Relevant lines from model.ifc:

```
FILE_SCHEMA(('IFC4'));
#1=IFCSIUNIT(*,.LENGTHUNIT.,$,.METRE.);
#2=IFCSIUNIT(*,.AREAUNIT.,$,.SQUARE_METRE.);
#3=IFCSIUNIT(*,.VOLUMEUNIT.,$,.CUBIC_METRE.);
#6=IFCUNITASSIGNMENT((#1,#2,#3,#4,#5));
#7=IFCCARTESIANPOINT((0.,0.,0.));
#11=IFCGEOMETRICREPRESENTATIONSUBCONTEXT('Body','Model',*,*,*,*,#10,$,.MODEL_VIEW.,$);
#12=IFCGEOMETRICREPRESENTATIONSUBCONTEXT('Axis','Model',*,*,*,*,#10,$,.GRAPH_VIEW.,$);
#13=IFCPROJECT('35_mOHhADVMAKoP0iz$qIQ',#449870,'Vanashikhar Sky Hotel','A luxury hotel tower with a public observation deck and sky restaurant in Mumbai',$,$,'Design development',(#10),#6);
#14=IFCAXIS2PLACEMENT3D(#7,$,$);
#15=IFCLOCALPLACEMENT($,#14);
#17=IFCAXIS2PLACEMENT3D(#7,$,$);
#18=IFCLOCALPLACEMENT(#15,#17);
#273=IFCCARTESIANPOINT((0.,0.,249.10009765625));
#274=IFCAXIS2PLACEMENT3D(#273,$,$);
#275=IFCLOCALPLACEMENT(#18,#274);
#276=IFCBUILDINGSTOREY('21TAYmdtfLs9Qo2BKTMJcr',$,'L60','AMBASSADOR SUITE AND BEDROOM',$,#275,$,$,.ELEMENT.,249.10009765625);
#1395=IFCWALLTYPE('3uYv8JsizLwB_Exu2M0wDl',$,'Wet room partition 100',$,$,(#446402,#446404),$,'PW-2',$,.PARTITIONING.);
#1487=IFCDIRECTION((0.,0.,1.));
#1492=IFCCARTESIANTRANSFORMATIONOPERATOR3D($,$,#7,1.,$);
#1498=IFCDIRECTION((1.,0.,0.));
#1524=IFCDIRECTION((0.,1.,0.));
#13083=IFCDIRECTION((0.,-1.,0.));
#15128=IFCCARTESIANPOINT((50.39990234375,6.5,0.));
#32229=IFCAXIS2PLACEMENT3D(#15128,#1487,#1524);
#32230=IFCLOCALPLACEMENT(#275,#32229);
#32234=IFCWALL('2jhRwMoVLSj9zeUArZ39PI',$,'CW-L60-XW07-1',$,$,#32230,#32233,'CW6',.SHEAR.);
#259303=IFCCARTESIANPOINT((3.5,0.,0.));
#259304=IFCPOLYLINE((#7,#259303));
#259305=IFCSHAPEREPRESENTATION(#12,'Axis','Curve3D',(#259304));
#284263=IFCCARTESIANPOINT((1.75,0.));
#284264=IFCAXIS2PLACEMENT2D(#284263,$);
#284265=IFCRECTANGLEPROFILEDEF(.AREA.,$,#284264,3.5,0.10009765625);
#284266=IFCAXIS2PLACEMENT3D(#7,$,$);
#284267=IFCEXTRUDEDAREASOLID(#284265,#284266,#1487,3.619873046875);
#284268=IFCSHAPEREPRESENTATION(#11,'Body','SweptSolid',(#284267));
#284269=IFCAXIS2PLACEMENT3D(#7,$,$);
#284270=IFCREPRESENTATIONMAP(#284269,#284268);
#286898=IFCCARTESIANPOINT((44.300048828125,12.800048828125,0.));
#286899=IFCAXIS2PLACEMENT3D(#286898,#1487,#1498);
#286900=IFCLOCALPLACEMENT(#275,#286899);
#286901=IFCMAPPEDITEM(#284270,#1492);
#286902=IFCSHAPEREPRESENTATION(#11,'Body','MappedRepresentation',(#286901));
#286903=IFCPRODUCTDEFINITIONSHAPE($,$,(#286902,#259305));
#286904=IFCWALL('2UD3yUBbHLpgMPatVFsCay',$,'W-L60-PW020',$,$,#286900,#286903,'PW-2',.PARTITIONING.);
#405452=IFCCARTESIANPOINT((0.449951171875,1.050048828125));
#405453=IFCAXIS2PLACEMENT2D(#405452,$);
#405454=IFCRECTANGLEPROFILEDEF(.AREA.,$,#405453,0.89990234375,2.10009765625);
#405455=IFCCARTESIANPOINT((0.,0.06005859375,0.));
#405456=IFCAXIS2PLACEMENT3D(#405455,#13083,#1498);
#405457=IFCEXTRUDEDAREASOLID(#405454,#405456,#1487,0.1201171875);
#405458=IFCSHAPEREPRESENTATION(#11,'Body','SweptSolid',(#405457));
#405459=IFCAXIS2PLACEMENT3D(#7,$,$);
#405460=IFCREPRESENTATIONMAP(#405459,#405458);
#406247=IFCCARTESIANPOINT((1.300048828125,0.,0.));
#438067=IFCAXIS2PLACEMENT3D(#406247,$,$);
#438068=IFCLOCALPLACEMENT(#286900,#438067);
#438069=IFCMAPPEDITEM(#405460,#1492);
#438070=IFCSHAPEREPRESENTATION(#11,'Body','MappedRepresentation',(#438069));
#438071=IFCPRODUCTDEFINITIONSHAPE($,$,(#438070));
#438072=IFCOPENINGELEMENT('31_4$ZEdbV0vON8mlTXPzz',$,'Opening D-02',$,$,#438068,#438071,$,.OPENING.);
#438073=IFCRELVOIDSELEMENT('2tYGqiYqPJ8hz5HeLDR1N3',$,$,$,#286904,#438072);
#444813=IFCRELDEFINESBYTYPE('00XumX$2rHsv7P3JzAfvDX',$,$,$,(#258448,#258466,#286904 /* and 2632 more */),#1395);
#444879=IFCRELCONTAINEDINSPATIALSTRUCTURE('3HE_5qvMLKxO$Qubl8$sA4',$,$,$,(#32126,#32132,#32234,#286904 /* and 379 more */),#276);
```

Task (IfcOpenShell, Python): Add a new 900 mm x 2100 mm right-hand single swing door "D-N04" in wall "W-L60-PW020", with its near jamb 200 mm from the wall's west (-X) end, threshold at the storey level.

```python
import numpy as np
import ifcopenshell
import ifcopenshell.api.feature
import ifcopenshell.api.geometry
import ifcopenshell.api.root
import ifcopenshell.api.spatial
import ifcopenshell.geom
import ifcopenshell.util.element
import ifcopenshell.util.placement
import ifcopenshell.util.representation
import ifcopenshell.util.shape
import ifcopenshell.util.unit

model = ifcopenshell.open("model.ifc")
unit_scale = ifcopenshell.util.unit.calculate_unit_scale(model)
settings = ifcopenshell.geom.settings()


def volume(element):
    """Net volume in cubic metres, openings subtracted."""
    shape = ifcopenshell.geom.create_shape(settings, element)
    return ifcopenshell.util.shape.get_volume(shape.geometry)


wall = model.by_guid("2UD3yUBbHLpgMPatVFsCay")
storey = ifcopenshell.util.element.get_container(wall, ifc_class="IfcBuildingStorey")
context = ifcopenshell.util.representation.get_context(model, "Model", "Body", "MODEL_VIEW")
before = volume(wall)

width, height, from_end, sill = 0.9, 2.1, 0.2, 0.0  # metres

# The wall runs along its own X axis, and the end named is its -X end.
wall_shape = ifcopenshell.geom.create_shape(settings, wall)
x, y, z = ifcopenshell.util.shape.get_vertices(wall_shape.geometry).T
start = x.min() + from_end
face, thickness = float(y.min()), float(y.max() - y.min())
wall_matrix = ifcopenshell.util.placement.get_local_placement(wall.ObjectPlacement)
level = ifcopenshell.util.placement.get_local_placement(storey.ObjectPlacement)[2, 3]


def in_wall(x, y):
    """Placement at x, y metres in the wall's axes, at sill height."""
    matrix = wall_matrix.copy()
    matrix[:, 3] = wall_matrix @ np.array([x / unit_scale, y / unit_scale, 0.0, 1.0])
    matrix[2, 3] = level + sill / unit_scale
    return matrix


# Opening: a box that overshoots both wall faces by 50 mm.
opening = ifcopenshell.api.root.create_entity(model, ifc_class="IfcOpeningElement", predefined_type="OPENING")
box = ifcopenshell.api.geometry.add_wall_representation(
    model, context=context, length=width, height=height, thickness=thickness + 0.1
)
ifcopenshell.api.geometry.assign_representation(model, product=opening, representation=box)
ifcopenshell.api.geometry.edit_object_placement(model, product=opening, matrix=in_wall(start, face - 0.05), is_si=False)
ifcopenshell.api.feature.add_feature(model, feature=opening, element=wall)

door = ifcopenshell.api.root.create_entity(model, ifc_class="IfcDoor", name="D-N04", predefined_type="DOOR")
door.OverallWidth, door.OverallHeight = width / unit_scale, height / unit_scale
door.OperationType = "SINGLE_SWING_RIGHT"
body = ifcopenshell.api.geometry.add_door_representation(
    model,
    context=context,
    overall_width=door.OverallWidth,
    overall_height=door.OverallHeight,
    operation_type="SINGLE_SWING_RIGHT",
    lining_properties={"LiningDepth": thickness / unit_scale, "ThresholdDepth": thickness / unit_scale},
)
ifcopenshell.api.geometry.assign_representation(model, product=door, representation=body)
ifcopenshell.api.spatial.assign_container(model, products=[door], relating_structure=storey)
ifcopenshell.api.feature.add_filling(model, opening=opening, element=door)

# The lining spans the wall, so the door starts at the wall face.
ifcopenshell.api.geometry.edit_object_placement(model, product=door, matrix=in_wall(start, face), is_si=False)

after = volume(wall)

print(f"wall volume {before:.3f} -> {after:.3f} m3")

model.write("model_edited.ifc")
```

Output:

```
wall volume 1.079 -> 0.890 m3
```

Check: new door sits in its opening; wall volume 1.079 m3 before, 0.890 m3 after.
